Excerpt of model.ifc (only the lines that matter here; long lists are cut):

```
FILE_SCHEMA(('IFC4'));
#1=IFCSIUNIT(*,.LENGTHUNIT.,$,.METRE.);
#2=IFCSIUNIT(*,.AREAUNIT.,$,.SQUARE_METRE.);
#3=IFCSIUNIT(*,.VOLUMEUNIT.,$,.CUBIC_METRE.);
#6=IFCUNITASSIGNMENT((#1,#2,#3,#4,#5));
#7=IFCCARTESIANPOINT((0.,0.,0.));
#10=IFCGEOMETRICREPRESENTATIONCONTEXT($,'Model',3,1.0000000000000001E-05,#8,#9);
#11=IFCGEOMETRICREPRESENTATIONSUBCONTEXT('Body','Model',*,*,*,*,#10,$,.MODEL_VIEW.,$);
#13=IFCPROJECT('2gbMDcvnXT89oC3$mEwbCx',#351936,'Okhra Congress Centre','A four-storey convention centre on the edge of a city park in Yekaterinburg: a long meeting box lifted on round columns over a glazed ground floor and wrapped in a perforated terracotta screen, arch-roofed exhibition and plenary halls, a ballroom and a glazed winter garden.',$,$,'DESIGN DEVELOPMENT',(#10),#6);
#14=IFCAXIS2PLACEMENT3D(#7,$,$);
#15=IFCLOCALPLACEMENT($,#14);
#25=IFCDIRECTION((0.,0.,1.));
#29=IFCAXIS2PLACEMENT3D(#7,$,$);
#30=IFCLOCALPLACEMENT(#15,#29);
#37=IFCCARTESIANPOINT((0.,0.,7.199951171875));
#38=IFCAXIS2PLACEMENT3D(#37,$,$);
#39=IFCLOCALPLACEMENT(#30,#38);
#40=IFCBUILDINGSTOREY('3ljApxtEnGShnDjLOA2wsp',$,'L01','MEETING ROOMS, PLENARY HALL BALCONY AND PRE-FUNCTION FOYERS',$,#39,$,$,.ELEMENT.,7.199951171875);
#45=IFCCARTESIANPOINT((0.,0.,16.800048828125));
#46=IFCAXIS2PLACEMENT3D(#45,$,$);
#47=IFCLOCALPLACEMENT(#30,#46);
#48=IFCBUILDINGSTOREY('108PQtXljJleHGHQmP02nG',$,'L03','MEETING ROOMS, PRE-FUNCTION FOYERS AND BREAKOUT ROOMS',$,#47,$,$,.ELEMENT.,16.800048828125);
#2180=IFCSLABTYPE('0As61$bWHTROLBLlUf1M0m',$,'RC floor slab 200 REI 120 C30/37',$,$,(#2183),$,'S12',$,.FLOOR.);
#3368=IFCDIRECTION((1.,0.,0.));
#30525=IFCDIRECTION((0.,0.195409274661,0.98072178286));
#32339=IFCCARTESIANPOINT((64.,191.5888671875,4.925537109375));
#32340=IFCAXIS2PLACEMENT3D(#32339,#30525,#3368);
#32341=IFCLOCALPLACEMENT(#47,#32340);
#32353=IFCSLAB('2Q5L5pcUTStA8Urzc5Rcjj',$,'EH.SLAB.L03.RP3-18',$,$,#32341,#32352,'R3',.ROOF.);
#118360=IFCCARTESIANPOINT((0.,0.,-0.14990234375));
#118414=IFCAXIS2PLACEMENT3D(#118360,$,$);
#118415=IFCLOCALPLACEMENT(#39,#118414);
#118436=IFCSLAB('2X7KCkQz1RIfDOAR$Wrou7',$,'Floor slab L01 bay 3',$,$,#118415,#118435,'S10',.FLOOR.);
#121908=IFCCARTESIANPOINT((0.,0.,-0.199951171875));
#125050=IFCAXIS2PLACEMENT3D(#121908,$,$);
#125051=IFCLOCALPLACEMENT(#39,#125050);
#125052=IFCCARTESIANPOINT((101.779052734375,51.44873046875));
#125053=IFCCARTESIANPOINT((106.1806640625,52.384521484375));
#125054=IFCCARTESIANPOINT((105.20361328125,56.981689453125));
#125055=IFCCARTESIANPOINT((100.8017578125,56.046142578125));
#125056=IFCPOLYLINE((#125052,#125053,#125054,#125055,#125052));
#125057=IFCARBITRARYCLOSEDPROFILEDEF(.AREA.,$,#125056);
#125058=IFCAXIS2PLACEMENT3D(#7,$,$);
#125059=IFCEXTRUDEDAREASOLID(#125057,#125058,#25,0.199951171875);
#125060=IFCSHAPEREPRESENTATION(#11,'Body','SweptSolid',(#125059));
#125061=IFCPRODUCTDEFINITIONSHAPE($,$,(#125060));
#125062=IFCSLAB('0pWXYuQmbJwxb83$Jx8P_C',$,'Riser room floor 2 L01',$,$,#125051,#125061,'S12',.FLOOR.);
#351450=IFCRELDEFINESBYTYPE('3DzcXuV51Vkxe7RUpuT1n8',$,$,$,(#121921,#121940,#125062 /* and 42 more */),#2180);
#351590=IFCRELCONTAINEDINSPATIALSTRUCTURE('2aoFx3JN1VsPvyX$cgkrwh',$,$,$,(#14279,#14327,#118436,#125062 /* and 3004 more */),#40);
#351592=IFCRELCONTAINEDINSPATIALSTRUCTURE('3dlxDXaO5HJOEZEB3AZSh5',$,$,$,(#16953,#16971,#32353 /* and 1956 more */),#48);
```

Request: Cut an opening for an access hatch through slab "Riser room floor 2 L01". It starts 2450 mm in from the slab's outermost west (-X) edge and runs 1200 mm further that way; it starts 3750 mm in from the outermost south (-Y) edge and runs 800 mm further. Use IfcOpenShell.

```python
import numpy as np
import ifcopenshell
import ifcopenshell.api.feature
import ifcopenshell.api.geometry
import ifcopenshell.api.root
import ifcopenshell.geom
import ifcopenshell.util.placement
import ifcopenshell.util.representation
import ifcopenshell.util.shape
import ifcopenshell.util.unit

model = ifcopenshell.open("model.ifc")
unit_scale = ifcopenshell.util.unit.calculate_unit_scale(model)
settings = ifcopenshell.geom.settings()


def volume(element):
    """Net volume in cubic metres, openings subtracted."""
    shape = ifcopenshell.geom.create_shape(settings, element)
    return ifcopenshell.util.shape.get_volume(shape.geometry)


slab = model.by_guid("0pWXYuQmbJwxb83$Jx8P_C")
before = volume(slab)

# Extent in the slab's own axes, in metres. The edges named are its -X and -Y sides.
slab_shape = ifcopenshell.geom.create_shape(settings, slab)
vertices = ifcopenshell.util.shape.get_vertices(slab_shape.geometry)
x_min, y_min, bottom = vertices.min(axis=0)
top = vertices[:, 2].max()

opening = ifcopenshell.api.root.create_entity(model, ifc_class="IfcOpeningElement", name="Access hatch opening", predefined_type="OPENING")
context = ifcopenshell.util.representation.get_context(model, "Model", "Body", "MODEL_VIEW")
width, depth = 1.2, 0.8
outline = [(0.0, 0.0), (width, 0.0), (width, depth), (0.0, depth), (0.0, 0.0)]
# Overshoot both faces by 50 mm so the cut is clean.
shape = ifcopenshell.api.geometry.add_slab_representation(
    model, context=context, depth=top - bottom + 0.1, polyline=outline
)
ifcopenshell.api.geometry.assign_representation(model, product=opening, representation=shape)

matrix = ifcopenshell.util.placement.get_local_placement(slab.ObjectPlacement)
matrix[:, 3] = matrix @ np.append(np.array([x_min + 2.45, y_min + 3.75, bottom - 0.05]) / unit_scale, 1.0)
ifcopenshell.api.geometry.edit_object_placement(model, product=opening, matrix=matrix, is_si=False)
ifcopenshell.api.feature.add_feature(model, feature=opening, element=slab)

after = volume(slab)

print(f"slab volume {before:.3f} -> {after:.3f} m3")

model.write("model-out.ifc")
```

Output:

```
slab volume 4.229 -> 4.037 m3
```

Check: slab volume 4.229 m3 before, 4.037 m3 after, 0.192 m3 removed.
